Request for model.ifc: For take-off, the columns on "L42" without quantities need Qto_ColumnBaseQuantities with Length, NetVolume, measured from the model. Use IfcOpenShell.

First a look at what the model holds.

```python
import ifcopenshell
import ifcopenshell.util.element
import ifcopenshell.util.unit

model = ifcopenshell.open("model.ifc")
print(model.schema)
for unit_type in ("LENGTHUNIT", "AREAUNIT", "VOLUMEUNIT"):
    print(unit_type, ifcopenshell.util.unit.calculate_unit_scale(model, unit_type))
storey = next(s for s in model.by_type("IfcBuildingStorey") if s.Name == "L42")
columns = [e for e in ifcopenshell.util.element.get_decomposition(storey) if e.is_a("IfcColumn")]
for e in sorted(columns, key=lambda e: e.id()):
    print(e.id(), e.is_a(), e.Name, list(ifcopenshell.util.element.get_psets(e, qtos_only=True)), sep=" | ")
```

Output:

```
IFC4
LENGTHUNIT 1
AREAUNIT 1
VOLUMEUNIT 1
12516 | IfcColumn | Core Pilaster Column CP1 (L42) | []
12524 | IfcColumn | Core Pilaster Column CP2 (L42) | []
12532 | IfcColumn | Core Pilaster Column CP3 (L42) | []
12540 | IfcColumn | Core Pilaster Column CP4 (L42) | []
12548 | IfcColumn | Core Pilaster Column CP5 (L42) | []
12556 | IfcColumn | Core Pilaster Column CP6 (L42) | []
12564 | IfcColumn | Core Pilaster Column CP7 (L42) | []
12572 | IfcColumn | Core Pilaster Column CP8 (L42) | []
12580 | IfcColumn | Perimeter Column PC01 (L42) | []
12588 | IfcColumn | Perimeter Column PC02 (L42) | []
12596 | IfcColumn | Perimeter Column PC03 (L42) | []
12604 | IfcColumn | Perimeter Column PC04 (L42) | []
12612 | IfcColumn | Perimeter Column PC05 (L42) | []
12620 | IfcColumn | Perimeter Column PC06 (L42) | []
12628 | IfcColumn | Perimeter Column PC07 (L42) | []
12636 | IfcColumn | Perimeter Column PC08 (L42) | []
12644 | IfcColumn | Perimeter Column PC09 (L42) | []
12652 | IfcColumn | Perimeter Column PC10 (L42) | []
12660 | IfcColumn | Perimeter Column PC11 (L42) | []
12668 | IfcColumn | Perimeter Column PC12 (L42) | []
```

```python
import ifcopenshell
import ifcopenshell.api.pset
import ifcopenshell.geom
import ifcopenshell.util.element
import ifcopenshell.util.shape
import ifcopenshell.util.unit

model = ifcopenshell.open("model.ifc")
unit_scale = ifcopenshell.util.unit.calculate_unit_scale(model)
volume_scale = ifcopenshell.util.unit.calculate_unit_scale(model, "VOLUMEUNIT")
settings = ifcopenshell.geom.settings()

storey = next(s for s in model.by_type("IfcBuildingStorey") if s.Name == "L42")
columns = [e for e in ifcopenshell.util.element.get_decomposition(storey) if e.is_a("IfcColumn")]

for e in sorted(columns, key=lambda e: e.id()):
    if ifcopenshell.util.element.get_psets(e, qtos_only=True, should_inherit=False):
        continue
    # Geometry comes back in metres, in the element's own axes.
    shape = ifcopenshell.geom.create_shape(settings, e)
    values = {
        "Length": ifcopenshell.util.shape.get_z(shape.geometry) / unit_scale,
        "NetVolume": ifcopenshell.util.shape.get_volume(shape.geometry) / volume_scale,
    }
    qto = ifcopenshell.api.pset.add_qto(model, product=e, name="Qto_ColumnBaseQuantities")
    ifcopenshell.api.pset.edit_qto(model, qto=qto, properties=values)
    print(e.id(), {k: round(v, 3) for k, v in values.items()})

model.write("model_v2.ifc")
```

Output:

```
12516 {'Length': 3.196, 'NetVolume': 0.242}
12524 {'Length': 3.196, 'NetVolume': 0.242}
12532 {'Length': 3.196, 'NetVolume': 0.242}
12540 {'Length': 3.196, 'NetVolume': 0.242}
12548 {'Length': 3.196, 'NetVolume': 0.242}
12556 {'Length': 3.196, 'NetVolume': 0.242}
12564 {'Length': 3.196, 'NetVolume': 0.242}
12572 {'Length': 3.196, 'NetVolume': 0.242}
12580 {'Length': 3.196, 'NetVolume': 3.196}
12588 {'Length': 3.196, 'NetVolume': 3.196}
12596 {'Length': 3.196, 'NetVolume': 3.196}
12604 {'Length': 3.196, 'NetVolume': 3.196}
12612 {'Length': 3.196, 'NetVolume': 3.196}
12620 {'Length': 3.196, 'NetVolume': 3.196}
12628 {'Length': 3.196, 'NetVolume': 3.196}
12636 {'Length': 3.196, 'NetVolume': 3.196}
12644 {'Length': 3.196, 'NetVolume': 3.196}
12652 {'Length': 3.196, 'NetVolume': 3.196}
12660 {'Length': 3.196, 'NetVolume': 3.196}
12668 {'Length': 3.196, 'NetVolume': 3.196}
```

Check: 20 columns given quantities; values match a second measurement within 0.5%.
